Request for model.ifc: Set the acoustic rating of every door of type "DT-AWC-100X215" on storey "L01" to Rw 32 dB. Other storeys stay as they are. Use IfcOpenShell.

First a look at what the model holds.

```python
import ifcopenshell
import ifcopenshell.util.element

model = ifcopenshell.open("model.ifc")
print(model.schema)
storey = next(s for s in model.by_type("IfcBuildingStorey") if s.Name == "L01")
doors = [e for e in ifcopenshell.util.element.get_decomposition(storey) if e.is_a("IfcDoor")]
seen = {}
for e in doors:
    element_type = ifcopenshell.util.element.get_type(e)
    key = (element_type.Name if element_type != e and element_type else None, ifcopenshell.util.element.get_pset(e, "Pset_DoorCommon", "AcousticRating"))
    seen[key] = seen.get(key, 0) + 1
for (name, value), count in sorted(seen.items(), key=str):
    print(count, "x", name, "|", value)
```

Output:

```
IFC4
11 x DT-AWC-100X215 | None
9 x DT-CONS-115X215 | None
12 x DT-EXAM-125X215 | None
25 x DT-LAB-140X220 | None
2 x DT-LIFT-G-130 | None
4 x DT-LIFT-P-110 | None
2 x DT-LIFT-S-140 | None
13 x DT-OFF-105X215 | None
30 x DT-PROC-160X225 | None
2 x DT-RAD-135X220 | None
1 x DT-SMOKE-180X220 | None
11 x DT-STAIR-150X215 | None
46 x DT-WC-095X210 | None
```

```python
import ifcopenshell
import ifcopenshell.api.pset
import ifcopenshell.util.element

model = ifcopenshell.open("model.ifc")

storey = next(s for s in model.by_type("IfcBuildingStorey") if s.Name == "L01")
doors = [e for e in ifcopenshell.util.element.get_decomposition(storey) if e.is_a("IfcDoor")]

count = 0
for e in doors:
    element_type = ifcopenshell.util.element.get_type(e)
    if element_type in (None, e) or element_type.Name != "DT-AWC-100X215":
        continue
    # add_pset returns the element's existing set when there is one.
    pset = ifcopenshell.api.pset.add_pset(model, product=e, name="Pset_DoorCommon")
    ifcopenshell.api.pset.edit_pset(model, pset=pset, properties={"AcousticRating": "Rw 32 dB"})
    count += 1

print(count, "doors updated")

model.write("model_v2.ifc")
```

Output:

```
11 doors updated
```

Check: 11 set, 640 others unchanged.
